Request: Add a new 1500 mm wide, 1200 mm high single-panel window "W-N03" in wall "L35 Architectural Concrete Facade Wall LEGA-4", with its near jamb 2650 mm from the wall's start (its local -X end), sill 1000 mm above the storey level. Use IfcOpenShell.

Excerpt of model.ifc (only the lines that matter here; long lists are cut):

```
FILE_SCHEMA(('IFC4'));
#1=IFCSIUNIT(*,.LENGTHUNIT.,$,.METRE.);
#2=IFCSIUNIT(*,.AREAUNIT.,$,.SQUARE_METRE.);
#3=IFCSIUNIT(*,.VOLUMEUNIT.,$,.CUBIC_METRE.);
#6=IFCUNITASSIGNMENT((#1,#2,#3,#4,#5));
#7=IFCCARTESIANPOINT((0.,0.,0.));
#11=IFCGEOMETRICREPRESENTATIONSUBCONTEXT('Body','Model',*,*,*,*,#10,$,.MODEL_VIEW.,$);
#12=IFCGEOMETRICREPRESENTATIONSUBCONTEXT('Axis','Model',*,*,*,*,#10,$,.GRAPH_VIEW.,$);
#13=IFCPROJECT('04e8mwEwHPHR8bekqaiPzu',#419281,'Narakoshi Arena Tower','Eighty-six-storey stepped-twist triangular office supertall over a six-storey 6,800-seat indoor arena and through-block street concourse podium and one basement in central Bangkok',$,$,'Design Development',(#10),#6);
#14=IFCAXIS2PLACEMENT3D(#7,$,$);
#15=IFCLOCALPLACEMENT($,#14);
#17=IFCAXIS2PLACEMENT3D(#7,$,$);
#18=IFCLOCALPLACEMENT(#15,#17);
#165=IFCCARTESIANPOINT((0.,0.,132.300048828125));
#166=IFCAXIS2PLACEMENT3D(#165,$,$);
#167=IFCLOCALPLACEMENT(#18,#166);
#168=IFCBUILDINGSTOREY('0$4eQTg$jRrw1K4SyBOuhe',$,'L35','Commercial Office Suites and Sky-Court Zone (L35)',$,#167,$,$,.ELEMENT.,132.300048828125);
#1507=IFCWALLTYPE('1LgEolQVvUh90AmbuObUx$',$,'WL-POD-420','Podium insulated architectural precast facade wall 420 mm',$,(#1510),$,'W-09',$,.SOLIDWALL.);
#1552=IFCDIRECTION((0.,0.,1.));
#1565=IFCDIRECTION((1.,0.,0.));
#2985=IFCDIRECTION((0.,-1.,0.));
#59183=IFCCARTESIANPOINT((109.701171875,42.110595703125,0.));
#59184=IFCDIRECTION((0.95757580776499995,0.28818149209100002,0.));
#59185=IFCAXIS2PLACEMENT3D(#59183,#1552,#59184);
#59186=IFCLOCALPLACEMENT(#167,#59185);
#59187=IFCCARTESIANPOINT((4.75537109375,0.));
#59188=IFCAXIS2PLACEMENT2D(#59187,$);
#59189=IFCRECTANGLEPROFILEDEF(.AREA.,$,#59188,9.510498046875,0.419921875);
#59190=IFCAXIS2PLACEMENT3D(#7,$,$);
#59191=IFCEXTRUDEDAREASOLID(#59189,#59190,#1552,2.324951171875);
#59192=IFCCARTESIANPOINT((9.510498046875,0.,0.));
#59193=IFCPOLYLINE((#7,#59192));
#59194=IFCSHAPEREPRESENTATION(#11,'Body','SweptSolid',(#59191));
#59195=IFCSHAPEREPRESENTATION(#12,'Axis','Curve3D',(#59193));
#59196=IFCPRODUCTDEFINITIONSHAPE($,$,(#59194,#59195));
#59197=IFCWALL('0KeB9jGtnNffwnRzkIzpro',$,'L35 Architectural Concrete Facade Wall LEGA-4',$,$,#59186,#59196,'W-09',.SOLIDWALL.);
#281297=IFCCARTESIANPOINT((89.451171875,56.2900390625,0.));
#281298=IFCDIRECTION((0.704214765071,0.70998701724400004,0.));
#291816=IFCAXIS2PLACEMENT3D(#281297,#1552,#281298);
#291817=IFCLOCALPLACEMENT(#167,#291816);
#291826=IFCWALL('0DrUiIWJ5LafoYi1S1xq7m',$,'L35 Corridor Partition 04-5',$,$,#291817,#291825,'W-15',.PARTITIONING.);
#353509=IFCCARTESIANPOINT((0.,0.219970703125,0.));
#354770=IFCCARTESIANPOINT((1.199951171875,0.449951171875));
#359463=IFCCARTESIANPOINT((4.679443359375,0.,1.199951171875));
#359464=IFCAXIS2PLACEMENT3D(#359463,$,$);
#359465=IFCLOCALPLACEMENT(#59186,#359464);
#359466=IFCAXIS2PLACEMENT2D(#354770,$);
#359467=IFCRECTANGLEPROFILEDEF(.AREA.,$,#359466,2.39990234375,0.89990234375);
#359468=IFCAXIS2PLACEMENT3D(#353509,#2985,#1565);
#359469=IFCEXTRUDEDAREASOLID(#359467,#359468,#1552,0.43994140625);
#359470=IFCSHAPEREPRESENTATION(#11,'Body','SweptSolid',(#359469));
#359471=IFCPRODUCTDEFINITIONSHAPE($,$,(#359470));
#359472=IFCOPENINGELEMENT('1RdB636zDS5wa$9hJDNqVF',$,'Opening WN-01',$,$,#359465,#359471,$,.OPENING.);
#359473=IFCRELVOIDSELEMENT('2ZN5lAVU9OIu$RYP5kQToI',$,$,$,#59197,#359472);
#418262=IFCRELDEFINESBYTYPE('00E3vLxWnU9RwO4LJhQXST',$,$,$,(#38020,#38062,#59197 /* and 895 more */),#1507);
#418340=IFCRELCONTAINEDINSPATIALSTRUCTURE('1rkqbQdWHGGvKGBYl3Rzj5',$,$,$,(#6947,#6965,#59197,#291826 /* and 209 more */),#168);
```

```python
import numpy as np
import ifcopenshell
import ifcopenshell.api.feature
import ifcopenshell.api.geometry
import ifcopenshell.api.root
import ifcopenshell.api.spatial
import ifcopenshell.geom
import ifcopenshell.util.element
import ifcopenshell.util.placement
import ifcopenshell.util.representation
import ifcopenshell.util.shape
import ifcopenshell.util.unit

model = ifcopenshell.open("model.ifc")
unit_scale = ifcopenshell.util.unit.calculate_unit_scale(model)
settings = ifcopenshell.geom.settings()


def volume(element):
    """Net volume in cubic metres, openings subtracted."""
    shape = ifcopenshell.geom.create_shape(settings, element)
    return ifcopenshell.util.shape.get_volume(shape.geometry)


wall = model.by_guid("0KeB9jGtnNffwnRzkIzpro")
storey = ifcopenshell.util.element.get_container(wall, ifc_class="IfcBuildingStorey")
context = ifcopenshell.util.representation.get_context(model, "Model", "Body", "MODEL_VIEW")
before = volume(wall)

width, height, from_end, sill = 1.5, 1.2, 2.65, 1  # metres

# The wall runs along its own X axis, and the end named is its -X end.
wall_shape = ifcopenshell.geom.create_shape(settings, wall)
x, y, z = ifcopenshell.util.shape.get_vertices(wall_shape.geometry).T
start = x.min() + from_end
face, thickness = float(y.min()), float(y.max() - y.min())
wall_matrix = ifcopenshell.util.placement.get_local_placement(wall.ObjectPlacement)
level = ifcopenshell.util.placement.get_local_placement(storey.ObjectPlacement)[2, 3]


def in_wall(x, y):
    """Placement at x, y metres in the wall's axes, at sill height."""
    matrix = wall_matrix.copy()
    matrix[:, 3] = wall_matrix @ np.array([x / unit_scale, y / unit_scale, 0.0, 1.0])
    matrix[2, 3] = level + sill / unit_scale
    return matrix


# Opening: a box that overshoots both wall faces by 50 mm.
opening = ifcopenshell.api.root.create_entity(model, ifc_class="IfcOpeningElement", predefined_type="OPENING")
box = ifcopenshell.api.geometry.add_wall_representation(
    model, context=context, length=width, height=height, thickness=thickness + 0.1
)
ifcopenshell.api.geometry.assign_representation(model, product=opening, representation=box)
ifcopenshell.api.geometry.edit_object_placement(model, product=opening, matrix=in_wall(start, face - 0.05), is_si=False)
ifcopenshell.api.feature.add_feature(model, feature=opening, element=wall)

window = ifcopenshell.api.root.create_entity(model, ifc_class="IfcWindow", name="W-N03", predefined_type="WINDOW")
window.OverallWidth, window.OverallHeight = width / unit_scale, height / unit_scale
window.PartitioningType = "SINGLE_PANEL"
body = ifcopenshell.api.geometry.add_window_representation(
    model,
    context=context,
    overall_width=window.OverallWidth,
    overall_height=window.OverallHeight,
    partition_type="SINGLE_PANEL",
)
ifcopenshell.api.geometry.assign_representation(model, product=window, representation=body)
ifcopenshell.api.spatial.assign_container(model, products=[window], relating_structure=storey)
ifcopenshell.api.feature.add_filling(model, opening=opening, element=window)

# Centre the window in the wall's thickness.
ifcopenshell.api.geometry.edit_object_placement(model, product=window, matrix=in_wall(start, face), is_si=False)
window_shape = ifcopenshell.geom.create_shape(settings, window)
depth = ifcopenshell.util.shape.get_vertices(window_shape.geometry)[:, 1]
offset = face + thickness / 2 - (depth.min() + depth.max()) / 2
ifcopenshell.api.geometry.edit_object_placement(model, product=window, matrix=in_wall(start, offset), is_si=False)

after = volume(wall)

print(f"wall volume {before:.3f} -> {after:.3f} m3")

model.write("model_rev.ifc")
```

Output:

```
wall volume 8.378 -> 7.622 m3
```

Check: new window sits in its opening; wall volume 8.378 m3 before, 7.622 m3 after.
